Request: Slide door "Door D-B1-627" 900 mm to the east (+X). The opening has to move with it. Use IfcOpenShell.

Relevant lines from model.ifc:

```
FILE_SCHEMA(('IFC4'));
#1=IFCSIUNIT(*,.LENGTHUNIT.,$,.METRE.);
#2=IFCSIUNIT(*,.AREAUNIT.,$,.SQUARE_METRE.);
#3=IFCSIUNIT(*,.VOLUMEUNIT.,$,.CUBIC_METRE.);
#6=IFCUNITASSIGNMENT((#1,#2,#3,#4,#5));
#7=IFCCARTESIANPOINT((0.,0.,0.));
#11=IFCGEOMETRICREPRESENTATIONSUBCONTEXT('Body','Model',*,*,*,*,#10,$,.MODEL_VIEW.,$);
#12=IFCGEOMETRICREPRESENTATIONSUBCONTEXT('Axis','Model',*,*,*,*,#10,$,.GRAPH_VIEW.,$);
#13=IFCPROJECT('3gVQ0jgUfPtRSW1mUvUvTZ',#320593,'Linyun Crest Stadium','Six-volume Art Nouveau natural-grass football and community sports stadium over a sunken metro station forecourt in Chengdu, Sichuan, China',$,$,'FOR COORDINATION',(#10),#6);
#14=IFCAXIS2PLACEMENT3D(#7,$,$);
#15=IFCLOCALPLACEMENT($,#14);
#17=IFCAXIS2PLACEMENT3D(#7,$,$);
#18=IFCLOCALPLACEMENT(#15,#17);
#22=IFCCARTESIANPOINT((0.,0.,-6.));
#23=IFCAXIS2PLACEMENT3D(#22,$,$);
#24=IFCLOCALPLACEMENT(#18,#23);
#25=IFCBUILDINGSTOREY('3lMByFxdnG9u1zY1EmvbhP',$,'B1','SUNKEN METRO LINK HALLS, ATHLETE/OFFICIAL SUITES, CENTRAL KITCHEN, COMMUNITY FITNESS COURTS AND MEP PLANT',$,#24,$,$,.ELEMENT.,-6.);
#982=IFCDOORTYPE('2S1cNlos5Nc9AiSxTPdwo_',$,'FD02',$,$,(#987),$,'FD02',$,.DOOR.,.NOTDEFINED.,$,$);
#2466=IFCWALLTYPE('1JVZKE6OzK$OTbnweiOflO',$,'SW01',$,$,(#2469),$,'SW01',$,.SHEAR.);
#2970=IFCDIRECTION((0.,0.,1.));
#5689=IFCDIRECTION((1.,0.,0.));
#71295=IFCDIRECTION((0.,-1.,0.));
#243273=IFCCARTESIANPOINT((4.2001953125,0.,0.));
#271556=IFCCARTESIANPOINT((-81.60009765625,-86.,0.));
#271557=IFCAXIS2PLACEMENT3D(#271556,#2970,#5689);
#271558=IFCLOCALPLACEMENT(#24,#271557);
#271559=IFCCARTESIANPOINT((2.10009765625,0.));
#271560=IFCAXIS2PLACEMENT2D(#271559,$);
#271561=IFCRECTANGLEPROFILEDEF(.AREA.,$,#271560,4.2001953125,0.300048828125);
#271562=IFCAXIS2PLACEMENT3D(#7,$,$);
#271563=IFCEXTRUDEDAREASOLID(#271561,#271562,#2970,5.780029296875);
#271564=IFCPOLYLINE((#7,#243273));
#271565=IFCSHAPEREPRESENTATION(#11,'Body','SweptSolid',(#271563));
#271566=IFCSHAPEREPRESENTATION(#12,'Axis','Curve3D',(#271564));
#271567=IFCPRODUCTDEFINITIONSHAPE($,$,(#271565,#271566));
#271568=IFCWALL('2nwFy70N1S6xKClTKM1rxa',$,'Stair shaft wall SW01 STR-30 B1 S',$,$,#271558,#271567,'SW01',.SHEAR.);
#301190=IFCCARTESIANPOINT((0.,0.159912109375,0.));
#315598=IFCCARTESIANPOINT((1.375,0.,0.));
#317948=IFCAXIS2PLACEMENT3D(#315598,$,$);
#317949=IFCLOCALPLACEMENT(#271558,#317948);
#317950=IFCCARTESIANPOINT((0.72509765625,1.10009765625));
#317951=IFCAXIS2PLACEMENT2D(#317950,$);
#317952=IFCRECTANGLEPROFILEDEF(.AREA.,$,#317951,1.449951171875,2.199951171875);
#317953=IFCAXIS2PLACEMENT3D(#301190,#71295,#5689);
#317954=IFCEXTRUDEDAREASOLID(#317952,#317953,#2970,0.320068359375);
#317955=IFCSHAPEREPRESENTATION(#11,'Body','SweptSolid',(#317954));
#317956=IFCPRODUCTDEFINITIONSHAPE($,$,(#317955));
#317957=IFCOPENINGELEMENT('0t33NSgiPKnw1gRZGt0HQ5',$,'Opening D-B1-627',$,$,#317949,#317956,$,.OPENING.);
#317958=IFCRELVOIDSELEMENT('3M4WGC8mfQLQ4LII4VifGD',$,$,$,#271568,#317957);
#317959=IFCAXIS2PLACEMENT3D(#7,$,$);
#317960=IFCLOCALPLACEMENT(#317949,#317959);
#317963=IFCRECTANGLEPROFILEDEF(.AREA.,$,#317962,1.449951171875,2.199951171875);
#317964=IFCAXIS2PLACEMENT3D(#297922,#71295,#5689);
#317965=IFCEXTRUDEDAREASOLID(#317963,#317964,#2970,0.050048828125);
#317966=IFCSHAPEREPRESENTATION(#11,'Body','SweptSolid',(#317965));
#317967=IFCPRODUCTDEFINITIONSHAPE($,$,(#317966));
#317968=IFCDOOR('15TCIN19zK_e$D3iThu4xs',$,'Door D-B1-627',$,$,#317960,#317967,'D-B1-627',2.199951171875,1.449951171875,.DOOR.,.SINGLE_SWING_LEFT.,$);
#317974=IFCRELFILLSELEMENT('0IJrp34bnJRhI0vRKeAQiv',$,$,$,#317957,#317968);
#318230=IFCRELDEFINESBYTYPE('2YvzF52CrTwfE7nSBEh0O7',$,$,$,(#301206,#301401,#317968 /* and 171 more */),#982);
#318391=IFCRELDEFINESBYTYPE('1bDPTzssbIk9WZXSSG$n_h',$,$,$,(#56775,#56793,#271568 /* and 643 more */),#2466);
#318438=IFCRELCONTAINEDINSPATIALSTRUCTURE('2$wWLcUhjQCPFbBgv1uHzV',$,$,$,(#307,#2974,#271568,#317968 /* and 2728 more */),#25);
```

```python
import ifcopenshell
import ifcopenshell.api.geometry
import ifcopenshell.util.placement
import ifcopenshell.util.unit

model = ifcopenshell.open("model.ifc")
unit_scale = ifcopenshell.util.unit.calculate_unit_scale(model)

door = model.by_guid("15TCIN19zK_e$D3iThu4xs")
opening = door.FillsVoids[0].RelatingOpeningElement
wall = opening.VoidsElements[0].RelatingBuildingElement

wall_matrix = ifcopenshell.util.placement.get_local_placement(wall.ObjectPlacement)
shift = wall_matrix[:3, 0] * 0.9 / unit_scale
before = ifcopenshell.util.placement.get_local_placement(door.ObjectPlacement)[:3, 3].copy()

# The door is placed relative to its opening, so it follows when the opening moves.
matrix = ifcopenshell.util.placement.get_local_placement(opening.ObjectPlacement)
matrix[:3, 3] += shift
ifcopenshell.api.geometry.edit_object_placement(
    model, product=opening, matrix=matrix, is_si=False, should_transform_children=True
)

after = ifcopenshell.util.placement.get_local_placement(door.ObjectPlacement)[:3, 3]
print("door moved by", (after - before).round(3) + 0.0)

model.write("model_v2.ifc")
```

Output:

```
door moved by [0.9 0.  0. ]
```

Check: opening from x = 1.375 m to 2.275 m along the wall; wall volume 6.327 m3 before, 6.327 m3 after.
